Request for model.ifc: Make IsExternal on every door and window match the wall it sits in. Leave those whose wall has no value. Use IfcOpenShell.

First a look at what the model holds.

```python
import ifcopenshell
import ifcopenshell.util.element

model = ifcopenshell.open("model.ifc")
print(model.schema)
seen = {}
for e in model.by_type("IfcDoor") + model.by_type("IfcWindow"):
    if not e.FillsVoids:
        continue
    host = e.FillsVoids[0].RelatingOpeningElement.VoidsElements[0].RelatingBuildingElement
    own = ifcopenshell.util.element.get_pset(e, f"Pset_{e.is_a()[3:].removesuffix('StandardCase')}Common", "IsExternal")
    wall = ifcopenshell.util.element.get_pset(host, "Pset_WallCommon", "IsExternal")
    seen[e.is_a(), own, wall] = seen.get((e.is_a(), own, wall), 0) + 1
for (cls, own, wall), count in sorted(seen.items(), key=str):
    print(count, cls, "IsExternal:", own, "| host wall:", wall)
```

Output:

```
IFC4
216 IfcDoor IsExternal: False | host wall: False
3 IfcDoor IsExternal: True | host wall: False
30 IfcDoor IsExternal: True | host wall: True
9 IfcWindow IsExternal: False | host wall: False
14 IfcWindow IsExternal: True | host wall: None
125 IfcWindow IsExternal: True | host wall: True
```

```python
import ifcopenshell
import ifcopenshell.api.pset
import ifcopenshell.util.element

model = ifcopenshell.open("model.ifc")

count = 0
for ifc_class, pset_name in (("IfcDoor", "Pset_DoorCommon"), ("IfcWindow", "Pset_WindowCommon")):
    for e in model.by_type(ifc_class):
        if not e.FillsVoids:
            continue
        host = e.FillsVoids[0].RelatingOpeningElement.VoidsElements[0].RelatingBuildingElement
        external = ifcopenshell.util.element.get_pset(host, "Pset_WallCommon", "IsExternal")
        if external is None or ifcopenshell.util.element.get_pset(e, pset_name, "IsExternal") == external:
            continue
        pset = ifcopenshell.api.pset.add_pset(model, product=e, name=pset_name)
        ifcopenshell.api.pset.edit_pset(model, pset=pset, properties={"IsExternal": external})
        count += 1

print(count, "updated")

model.write("model-out.ifc")
```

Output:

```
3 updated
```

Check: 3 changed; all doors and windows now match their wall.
